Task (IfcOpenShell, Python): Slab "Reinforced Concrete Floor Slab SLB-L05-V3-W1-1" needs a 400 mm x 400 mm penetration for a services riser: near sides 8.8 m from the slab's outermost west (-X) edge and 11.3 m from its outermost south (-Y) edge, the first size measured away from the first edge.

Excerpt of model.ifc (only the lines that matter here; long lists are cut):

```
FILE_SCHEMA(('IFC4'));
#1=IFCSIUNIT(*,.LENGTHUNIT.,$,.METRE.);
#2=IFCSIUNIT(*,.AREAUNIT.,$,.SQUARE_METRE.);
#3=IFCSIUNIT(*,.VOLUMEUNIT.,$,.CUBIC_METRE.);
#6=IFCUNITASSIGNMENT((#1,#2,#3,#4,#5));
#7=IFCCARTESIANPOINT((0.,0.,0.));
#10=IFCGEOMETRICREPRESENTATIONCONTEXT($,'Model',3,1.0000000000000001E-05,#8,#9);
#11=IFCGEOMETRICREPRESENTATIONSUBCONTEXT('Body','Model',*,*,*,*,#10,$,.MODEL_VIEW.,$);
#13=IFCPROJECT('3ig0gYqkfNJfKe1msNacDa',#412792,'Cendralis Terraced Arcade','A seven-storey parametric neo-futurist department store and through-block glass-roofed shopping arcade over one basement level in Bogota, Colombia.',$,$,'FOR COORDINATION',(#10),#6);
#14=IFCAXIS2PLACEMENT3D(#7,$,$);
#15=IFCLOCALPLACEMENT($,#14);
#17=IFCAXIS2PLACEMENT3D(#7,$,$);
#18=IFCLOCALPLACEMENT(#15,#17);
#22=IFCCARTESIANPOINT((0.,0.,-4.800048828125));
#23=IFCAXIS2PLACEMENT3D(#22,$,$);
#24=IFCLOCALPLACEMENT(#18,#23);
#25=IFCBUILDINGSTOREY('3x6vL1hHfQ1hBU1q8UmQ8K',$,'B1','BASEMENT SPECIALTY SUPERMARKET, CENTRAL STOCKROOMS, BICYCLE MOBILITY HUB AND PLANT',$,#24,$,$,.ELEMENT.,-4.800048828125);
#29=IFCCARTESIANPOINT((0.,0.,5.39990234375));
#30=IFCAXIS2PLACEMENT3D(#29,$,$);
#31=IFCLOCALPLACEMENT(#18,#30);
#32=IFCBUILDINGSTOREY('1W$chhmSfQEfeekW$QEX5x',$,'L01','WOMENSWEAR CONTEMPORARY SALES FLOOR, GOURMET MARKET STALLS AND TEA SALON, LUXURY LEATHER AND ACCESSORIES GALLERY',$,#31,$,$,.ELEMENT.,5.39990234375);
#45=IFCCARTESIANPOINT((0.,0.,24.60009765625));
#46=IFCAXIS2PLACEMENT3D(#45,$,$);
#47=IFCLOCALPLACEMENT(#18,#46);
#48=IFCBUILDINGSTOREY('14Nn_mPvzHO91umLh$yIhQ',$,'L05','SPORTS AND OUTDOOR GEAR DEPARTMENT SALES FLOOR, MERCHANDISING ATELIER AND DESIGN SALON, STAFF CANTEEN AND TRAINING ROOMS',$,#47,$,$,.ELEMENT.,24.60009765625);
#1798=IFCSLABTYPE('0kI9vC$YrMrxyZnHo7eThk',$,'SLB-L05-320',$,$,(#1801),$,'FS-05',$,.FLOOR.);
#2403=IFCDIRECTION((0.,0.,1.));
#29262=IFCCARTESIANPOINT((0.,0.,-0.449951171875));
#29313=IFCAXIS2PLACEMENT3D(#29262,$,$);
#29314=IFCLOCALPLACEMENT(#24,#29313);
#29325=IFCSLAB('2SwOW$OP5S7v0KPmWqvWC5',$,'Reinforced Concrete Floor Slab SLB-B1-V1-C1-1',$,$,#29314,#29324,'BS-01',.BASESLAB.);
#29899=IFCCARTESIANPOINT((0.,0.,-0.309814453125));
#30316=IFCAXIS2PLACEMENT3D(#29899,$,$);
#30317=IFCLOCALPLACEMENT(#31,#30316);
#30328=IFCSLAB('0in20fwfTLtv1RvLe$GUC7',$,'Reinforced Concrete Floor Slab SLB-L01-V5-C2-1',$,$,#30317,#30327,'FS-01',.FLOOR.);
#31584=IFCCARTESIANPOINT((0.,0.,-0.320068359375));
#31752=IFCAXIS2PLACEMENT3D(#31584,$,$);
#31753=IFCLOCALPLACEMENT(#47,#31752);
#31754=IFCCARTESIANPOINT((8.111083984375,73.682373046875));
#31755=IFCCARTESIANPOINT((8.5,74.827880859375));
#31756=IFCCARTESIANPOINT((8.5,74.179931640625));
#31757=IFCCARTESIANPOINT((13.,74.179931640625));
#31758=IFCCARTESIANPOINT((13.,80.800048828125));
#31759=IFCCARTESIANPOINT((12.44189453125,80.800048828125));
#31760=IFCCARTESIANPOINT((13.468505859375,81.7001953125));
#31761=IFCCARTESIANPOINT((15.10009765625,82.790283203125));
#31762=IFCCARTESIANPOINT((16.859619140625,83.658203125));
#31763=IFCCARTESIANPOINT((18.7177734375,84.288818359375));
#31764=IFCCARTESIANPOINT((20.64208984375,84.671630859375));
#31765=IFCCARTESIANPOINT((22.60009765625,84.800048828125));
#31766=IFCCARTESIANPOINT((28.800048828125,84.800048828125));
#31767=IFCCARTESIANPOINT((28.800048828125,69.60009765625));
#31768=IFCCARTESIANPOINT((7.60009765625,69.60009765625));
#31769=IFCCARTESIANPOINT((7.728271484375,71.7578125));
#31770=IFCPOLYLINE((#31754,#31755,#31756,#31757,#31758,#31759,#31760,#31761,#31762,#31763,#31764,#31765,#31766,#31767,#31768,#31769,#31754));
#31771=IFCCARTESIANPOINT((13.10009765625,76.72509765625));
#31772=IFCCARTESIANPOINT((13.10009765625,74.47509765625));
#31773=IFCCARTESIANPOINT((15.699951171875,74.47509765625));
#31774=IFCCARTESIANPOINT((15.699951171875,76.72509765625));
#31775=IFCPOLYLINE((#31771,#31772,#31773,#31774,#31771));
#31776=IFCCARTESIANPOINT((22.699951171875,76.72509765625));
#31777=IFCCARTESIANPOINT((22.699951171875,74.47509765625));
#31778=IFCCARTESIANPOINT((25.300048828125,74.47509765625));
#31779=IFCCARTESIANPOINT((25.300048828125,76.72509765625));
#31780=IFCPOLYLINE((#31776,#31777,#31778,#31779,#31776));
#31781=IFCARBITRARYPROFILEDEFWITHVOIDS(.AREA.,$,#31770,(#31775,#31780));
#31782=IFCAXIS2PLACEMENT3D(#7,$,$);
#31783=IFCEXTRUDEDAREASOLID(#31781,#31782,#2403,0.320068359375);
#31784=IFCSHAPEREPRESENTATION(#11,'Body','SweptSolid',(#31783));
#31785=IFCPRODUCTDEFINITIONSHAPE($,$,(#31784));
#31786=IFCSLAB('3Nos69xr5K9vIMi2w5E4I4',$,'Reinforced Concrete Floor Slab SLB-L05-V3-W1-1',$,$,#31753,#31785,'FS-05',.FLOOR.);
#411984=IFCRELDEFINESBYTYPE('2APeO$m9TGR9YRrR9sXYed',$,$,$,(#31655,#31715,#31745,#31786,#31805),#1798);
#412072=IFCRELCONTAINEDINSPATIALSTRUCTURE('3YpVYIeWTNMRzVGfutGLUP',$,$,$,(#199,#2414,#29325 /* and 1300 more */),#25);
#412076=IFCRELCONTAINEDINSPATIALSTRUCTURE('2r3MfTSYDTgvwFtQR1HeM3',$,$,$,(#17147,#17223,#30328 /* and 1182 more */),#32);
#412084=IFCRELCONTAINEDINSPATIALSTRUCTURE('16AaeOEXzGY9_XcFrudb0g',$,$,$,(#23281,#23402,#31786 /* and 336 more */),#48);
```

```python
import numpy as np
import ifcopenshell
import ifcopenshell.api.feature
import ifcopenshell.api.geometry
import ifcopenshell.api.root
import ifcopenshell.geom
import ifcopenshell.util.placement
import ifcopenshell.util.representation
import ifcopenshell.util.shape
import ifcopenshell.util.unit

model = ifcopenshell.open("model.ifc")
unit_scale = ifcopenshell.util.unit.calculate_unit_scale(model)
settings = ifcopenshell.geom.settings()


def volume(element):
    """Net volume in cubic metres, openings subtracted."""
    shape = ifcopenshell.geom.create_shape(settings, element)
    return ifcopenshell.util.shape.get_volume(shape.geometry)


slab = model.by_guid("3Nos69xr5K9vIMi2w5E4I4")
before = volume(slab)

# Extent in the slab's own axes, in metres. The edges named are its -X and -Y sides.
slab_shape = ifcopenshell.geom.create_shape(settings, slab)
vertices = ifcopenshell.util.shape.get_vertices(slab_shape.geometry)
x_min, y_min, bottom = vertices.min(axis=0)
top = vertices[:, 2].max()

opening = ifcopenshell.api.root.create_entity(model, ifc_class="IfcOpeningElement", name="Services riser opening", predefined_type="OPENING")
context = ifcopenshell.util.representation.get_context(model, "Model", "Body", "MODEL_VIEW")
width, depth = 0.4, 0.4
outline = [(0.0, 0.0), (width, 0.0), (width, depth), (0.0, depth), (0.0, 0.0)]
# Overshoot both faces by 50 mm so the cut is clean.
shape = ifcopenshell.api.geometry.add_slab_representation(
    model, context=context, depth=top - bottom + 0.1, polyline=outline
)
ifcopenshell.api.geometry.assign_representation(model, product=opening, representation=shape)

matrix = ifcopenshell.util.placement.get_local_placement(slab.ObjectPlacement)
matrix[:, 3] = matrix @ np.append(np.array([x_min + 8.8, y_min + 11.3, bottom - 0.05]) / unit_scale, 1.0)
ifcopenshell.api.geometry.edit_object_placement(model, product=opening, matrix=matrix, is_si=False)
ifcopenshell.api.feature.add_feature(model, feature=opening, element=slab)

after = volume(slab)

print(f"slab volume {before:.3f} -> {after:.3f} m3")

model.write("model_v2.ifc")
```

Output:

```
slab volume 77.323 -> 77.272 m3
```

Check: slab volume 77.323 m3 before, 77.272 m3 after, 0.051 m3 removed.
